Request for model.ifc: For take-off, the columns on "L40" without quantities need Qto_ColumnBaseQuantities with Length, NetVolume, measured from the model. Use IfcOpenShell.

First a look at what the model holds.

```python
import ifcopenshell
import ifcopenshell.util.element
import ifcopenshell.util.unit

model = ifcopenshell.open("model.ifc")
print(model.schema)
for unit_type in ("LENGTHUNIT", "AREAUNIT", "VOLUMEUNIT"):
    print(unit_type, ifcopenshell.util.unit.calculate_unit_scale(model, unit_type))
storey = next(s for s in model.by_type("IfcBuildingStorey") if s.Name == "L40")
columns = [e for e in ifcopenshell.util.element.get_decomposition(storey) if e.is_a("IfcColumn")]
for e in sorted(columns, key=lambda e: e.id()):
    print(e.id(), e.is_a(), e.Name, list(ifcopenshell.util.element.get_psets(e, qtos_only=True)), sep=" | ")
```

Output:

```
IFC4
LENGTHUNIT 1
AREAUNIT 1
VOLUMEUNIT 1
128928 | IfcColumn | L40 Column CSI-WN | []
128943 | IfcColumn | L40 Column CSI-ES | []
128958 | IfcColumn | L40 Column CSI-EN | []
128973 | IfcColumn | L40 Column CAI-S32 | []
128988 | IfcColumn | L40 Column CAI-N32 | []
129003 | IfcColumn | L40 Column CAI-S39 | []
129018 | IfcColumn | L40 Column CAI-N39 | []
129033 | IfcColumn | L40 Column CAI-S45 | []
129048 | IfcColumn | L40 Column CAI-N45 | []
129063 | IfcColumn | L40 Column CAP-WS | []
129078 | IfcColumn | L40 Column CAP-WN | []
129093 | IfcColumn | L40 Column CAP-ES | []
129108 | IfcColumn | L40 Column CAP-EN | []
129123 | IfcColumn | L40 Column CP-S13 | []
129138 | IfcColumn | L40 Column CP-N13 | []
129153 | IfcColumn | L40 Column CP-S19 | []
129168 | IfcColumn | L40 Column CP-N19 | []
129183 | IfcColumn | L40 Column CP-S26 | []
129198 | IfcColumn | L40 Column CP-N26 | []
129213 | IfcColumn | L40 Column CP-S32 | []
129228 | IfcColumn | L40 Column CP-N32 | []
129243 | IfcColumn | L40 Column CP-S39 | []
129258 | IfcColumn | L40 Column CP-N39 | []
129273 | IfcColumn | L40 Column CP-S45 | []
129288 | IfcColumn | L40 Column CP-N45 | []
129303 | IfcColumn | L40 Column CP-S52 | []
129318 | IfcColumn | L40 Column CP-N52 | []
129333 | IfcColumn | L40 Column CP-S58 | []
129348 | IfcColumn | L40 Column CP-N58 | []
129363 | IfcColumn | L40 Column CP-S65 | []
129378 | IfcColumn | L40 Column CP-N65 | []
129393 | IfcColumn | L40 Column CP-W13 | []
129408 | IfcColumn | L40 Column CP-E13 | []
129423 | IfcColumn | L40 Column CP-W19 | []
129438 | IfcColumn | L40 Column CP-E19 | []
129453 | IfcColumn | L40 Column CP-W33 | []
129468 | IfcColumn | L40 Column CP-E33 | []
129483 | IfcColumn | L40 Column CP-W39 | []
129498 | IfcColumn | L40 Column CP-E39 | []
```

```python
import ifcopenshell
import ifcopenshell.api.pset
import ifcopenshell.geom
import ifcopenshell.util.element
import ifcopenshell.util.shape
import ifcopenshell.util.unit

model = ifcopenshell.open("model.ifc")
unit_scale = ifcopenshell.util.unit.calculate_unit_scale(model)
volume_scale = ifcopenshell.util.unit.calculate_unit_scale(model, "VOLUMEUNIT")
settings = ifcopenshell.geom.settings()

storey = next(s for s in model.by_type("IfcBuildingStorey") if s.Name == "L40")
columns = [e for e in ifcopenshell.util.element.get_decomposition(storey) if e.is_a("IfcColumn")]

for e in sorted(columns, key=lambda e: e.id()):
    if ifcopenshell.util.element.get_psets(e, qtos_only=True, should_inherit=False):
        continue
    # Geometry comes back in metres, in the element's own axes.
    shape = ifcopenshell.geom.create_shape(settings, e)
    values = {
        "Length": ifcopenshell.util.shape.get_z(shape.geometry) / unit_scale,
        "NetVolume": ifcopenshell.util.shape.get_volume(shape.geometry) / volume_scale,
    }
    qto = ifcopenshell.api.pset.add_qto(model, product=e, name="Qto_ColumnBaseQuantities")
    ifcopenshell.api.pset.edit_qto(model, qto=qto, properties=values)
    print(e.id(), {k: round(v, 3) for k, v in values.items()})

model.write("model_edited.ifc")
```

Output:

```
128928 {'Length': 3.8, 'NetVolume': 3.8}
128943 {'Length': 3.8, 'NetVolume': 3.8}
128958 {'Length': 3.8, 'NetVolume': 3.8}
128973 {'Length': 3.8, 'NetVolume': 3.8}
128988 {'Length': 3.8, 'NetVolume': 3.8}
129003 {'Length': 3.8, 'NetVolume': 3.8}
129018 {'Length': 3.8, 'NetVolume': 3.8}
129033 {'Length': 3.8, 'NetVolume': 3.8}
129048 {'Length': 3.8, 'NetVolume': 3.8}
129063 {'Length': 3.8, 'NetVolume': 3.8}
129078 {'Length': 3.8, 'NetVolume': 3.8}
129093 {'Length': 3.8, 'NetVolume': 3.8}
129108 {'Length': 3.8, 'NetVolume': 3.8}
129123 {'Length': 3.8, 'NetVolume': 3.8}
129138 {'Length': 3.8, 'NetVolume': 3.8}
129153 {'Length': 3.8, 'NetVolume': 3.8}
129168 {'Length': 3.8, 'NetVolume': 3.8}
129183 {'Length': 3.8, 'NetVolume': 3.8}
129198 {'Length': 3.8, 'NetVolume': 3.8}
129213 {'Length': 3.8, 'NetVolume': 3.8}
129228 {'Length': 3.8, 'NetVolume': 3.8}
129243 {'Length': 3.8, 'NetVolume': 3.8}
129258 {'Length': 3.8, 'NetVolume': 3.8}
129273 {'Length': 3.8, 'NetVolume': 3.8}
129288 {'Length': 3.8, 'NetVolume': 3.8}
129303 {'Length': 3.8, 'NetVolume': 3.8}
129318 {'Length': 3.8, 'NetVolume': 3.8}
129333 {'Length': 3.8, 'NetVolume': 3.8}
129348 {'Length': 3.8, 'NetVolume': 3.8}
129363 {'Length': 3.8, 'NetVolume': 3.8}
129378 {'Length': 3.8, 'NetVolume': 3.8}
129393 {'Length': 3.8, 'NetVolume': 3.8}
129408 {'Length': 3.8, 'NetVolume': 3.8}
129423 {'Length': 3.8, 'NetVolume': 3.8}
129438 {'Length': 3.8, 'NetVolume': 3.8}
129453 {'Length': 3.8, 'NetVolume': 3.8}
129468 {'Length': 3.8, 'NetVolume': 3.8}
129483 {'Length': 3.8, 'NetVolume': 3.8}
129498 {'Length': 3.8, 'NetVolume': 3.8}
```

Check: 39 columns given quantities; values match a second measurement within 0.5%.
